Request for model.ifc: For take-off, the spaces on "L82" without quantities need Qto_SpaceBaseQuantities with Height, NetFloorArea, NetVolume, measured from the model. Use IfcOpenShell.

First a look at what the model holds.

```python
import ifcopenshell
import ifcopenshell.util.element
import ifcopenshell.util.unit

model = ifcopenshell.open("model.ifc")
print(model.schema)
for unit_type in ("LENGTHUNIT", "AREAUNIT", "VOLUMEUNIT"):
    print(unit_type, ifcopenshell.util.unit.calculate_unit_scale(model, unit_type))
storey = next(s for s in model.by_type("IfcBuildingStorey") if s.Name == "L82")
spaces = [e for e in ifcopenshell.util.element.get_decomposition(storey) if e.is_a("IfcSpace")]
for e in sorted(spaces, key=lambda e: e.id()):
    print(e.id(), e.is_a(), e.Name, list(ifcopenshell.util.element.get_psets(e, qtos_only=True)), sep=" | ")
```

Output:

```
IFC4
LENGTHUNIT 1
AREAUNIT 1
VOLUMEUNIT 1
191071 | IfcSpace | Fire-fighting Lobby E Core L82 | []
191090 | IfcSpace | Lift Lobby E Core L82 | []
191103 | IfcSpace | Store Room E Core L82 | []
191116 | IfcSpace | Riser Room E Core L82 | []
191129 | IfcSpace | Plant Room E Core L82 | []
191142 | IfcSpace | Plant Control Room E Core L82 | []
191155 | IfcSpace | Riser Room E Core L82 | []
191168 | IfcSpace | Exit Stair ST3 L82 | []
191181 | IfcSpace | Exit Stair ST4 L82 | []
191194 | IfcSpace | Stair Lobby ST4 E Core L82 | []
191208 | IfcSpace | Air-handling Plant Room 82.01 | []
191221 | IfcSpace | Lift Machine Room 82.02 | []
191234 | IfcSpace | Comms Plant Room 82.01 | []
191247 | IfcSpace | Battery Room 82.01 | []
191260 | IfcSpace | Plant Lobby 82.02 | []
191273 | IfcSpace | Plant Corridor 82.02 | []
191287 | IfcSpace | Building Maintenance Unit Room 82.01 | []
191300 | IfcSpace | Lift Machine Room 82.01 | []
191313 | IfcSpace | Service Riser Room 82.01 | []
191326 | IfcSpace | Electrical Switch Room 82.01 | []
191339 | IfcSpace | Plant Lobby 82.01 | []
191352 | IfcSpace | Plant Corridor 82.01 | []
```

```python
import ifcopenshell
import ifcopenshell.api.pset
import ifcopenshell.geom
import ifcopenshell.util.element
import ifcopenshell.util.shape
import ifcopenshell.util.unit

model = ifcopenshell.open("model.ifc")
unit_scale = ifcopenshell.util.unit.calculate_unit_scale(model)
area_scale = ifcopenshell.util.unit.calculate_unit_scale(model, "AREAUNIT")
volume_scale = ifcopenshell.util.unit.calculate_unit_scale(model, "VOLUMEUNIT")
settings = ifcopenshell.geom.settings()

storey = next(s for s in model.by_type("IfcBuildingStorey") if s.Name == "L82")
spaces = [e for e in ifcopenshell.util.element.get_decomposition(storey) if e.is_a("IfcSpace")]

for e in sorted(spaces, key=lambda e: e.id()):
    if ifcopenshell.util.element.get_psets(e, qtos_only=True, should_inherit=False):
        continue
    # Geometry comes back in metres, in the element's own axes.
    shape = ifcopenshell.geom.create_shape(settings, e)
    values = {
        "Height": ifcopenshell.util.shape.get_z(shape.geometry) / unit_scale,
        "NetFloorArea": ifcopenshell.util.shape.get_footprint_area(shape.geometry) / area_scale,
        "NetVolume": ifcopenshell.util.shape.get_volume(shape.geometry) / volume_scale,
    }
    qto = ifcopenshell.api.pset.add_qto(model, product=e, name="Qto_SpaceBaseQuantities")
    ifcopenshell.api.pset.edit_qto(model, qto=qto, properties=values)
    print(e.id(), {k: round(v, 3) for k, v in values.items()})

model.write("model_edited.ifc")
```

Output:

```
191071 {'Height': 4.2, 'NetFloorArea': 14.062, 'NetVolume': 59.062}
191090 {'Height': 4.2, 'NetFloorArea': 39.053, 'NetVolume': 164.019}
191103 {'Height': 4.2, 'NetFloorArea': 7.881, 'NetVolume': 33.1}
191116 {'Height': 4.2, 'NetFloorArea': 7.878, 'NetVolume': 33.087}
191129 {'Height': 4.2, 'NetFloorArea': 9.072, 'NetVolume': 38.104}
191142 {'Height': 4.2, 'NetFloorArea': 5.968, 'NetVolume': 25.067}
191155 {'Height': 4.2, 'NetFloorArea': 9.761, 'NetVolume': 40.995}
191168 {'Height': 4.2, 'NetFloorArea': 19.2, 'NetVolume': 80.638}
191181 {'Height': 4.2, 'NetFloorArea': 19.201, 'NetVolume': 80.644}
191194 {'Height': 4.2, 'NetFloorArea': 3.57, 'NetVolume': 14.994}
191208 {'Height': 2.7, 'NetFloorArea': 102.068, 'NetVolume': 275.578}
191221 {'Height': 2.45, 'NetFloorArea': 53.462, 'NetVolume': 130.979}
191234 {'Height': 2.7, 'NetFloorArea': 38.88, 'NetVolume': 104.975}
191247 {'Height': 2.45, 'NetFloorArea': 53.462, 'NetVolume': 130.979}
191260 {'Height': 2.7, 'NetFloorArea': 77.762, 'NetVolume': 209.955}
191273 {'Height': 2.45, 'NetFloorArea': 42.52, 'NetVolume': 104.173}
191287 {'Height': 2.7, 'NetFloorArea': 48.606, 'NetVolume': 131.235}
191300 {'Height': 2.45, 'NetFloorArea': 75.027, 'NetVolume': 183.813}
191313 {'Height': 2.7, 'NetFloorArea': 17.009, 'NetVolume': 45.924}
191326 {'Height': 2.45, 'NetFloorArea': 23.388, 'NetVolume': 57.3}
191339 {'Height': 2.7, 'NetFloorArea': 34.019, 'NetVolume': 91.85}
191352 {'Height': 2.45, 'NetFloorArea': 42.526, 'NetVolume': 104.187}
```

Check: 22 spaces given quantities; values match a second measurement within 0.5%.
